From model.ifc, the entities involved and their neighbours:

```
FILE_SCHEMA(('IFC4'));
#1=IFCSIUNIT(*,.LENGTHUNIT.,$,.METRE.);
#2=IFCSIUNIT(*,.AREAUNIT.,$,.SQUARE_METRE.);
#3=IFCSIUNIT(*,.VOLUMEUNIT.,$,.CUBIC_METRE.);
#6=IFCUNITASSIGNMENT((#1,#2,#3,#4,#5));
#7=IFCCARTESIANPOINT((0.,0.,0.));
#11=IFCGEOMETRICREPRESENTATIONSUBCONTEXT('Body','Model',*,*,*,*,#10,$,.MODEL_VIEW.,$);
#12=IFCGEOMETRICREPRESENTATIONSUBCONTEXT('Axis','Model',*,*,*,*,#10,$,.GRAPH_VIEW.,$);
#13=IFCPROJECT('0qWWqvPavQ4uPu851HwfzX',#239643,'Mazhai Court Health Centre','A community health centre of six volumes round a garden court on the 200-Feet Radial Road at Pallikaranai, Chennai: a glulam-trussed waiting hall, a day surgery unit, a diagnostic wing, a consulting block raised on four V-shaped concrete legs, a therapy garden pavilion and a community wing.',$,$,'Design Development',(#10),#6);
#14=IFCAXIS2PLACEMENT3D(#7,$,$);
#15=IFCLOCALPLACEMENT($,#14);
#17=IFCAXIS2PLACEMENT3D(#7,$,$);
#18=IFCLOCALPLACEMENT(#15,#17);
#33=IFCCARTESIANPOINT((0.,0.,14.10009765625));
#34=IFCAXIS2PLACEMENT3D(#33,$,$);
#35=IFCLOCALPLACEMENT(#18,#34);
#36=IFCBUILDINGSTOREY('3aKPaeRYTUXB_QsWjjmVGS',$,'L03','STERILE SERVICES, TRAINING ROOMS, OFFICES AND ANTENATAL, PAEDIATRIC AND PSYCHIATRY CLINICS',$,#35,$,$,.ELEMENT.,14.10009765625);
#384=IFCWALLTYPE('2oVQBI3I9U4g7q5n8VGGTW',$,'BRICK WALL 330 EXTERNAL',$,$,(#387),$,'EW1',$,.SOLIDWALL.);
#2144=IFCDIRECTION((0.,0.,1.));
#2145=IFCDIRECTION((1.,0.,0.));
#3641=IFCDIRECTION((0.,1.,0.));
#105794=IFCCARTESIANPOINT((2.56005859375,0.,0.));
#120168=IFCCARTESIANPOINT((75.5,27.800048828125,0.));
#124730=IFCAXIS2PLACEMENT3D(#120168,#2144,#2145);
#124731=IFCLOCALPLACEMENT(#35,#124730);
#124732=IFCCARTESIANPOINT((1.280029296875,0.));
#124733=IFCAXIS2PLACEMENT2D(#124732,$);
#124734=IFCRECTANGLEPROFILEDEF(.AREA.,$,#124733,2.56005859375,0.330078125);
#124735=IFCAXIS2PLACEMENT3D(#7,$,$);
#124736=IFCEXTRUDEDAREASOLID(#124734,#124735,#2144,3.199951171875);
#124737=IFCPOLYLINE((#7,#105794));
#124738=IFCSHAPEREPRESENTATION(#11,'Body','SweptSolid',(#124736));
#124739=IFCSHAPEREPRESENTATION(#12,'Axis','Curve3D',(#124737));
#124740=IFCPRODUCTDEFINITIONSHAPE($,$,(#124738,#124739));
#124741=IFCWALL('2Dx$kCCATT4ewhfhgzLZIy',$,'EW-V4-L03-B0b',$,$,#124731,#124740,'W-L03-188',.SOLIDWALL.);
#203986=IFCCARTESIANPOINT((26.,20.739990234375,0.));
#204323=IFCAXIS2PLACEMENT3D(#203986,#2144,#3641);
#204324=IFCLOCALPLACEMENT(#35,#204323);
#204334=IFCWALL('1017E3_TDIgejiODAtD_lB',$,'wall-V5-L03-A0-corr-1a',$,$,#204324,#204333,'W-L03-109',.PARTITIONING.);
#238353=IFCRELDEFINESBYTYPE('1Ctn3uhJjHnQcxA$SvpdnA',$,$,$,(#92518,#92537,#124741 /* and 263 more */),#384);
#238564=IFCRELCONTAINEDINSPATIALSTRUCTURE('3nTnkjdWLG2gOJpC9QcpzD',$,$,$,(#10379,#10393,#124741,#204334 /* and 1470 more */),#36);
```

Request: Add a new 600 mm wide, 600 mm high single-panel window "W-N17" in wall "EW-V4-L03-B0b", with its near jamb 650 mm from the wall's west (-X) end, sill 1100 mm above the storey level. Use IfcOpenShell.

```python
import numpy as np
import ifcopenshell
import ifcopenshell.api.feature
import ifcopenshell.api.geometry
import ifcopenshell.api.root
import ifcopenshell.api.spatial
import ifcopenshell.geom
import ifcopenshell.util.element
import ifcopenshell.util.placement
import ifcopenshell.util.representation
import ifcopenshell.util.shape
import ifcopenshell.util.unit

model = ifcopenshell.open("model.ifc")
unit_scale = ifcopenshell.util.unit.calculate_unit_scale(model)
settings = ifcopenshell.geom.settings()


def volume(element):
    """Net volume in cubic metres, openings subtracted."""
    shape = ifcopenshell.geom.create_shape(settings, element)
    return ifcopenshell.util.shape.get_volume(shape.geometry)


wall = model.by_id(124741)
storey = ifcopenshell.util.element.get_container(wall, ifc_class="IfcBuildingStorey")
context = ifcopenshell.util.representation.get_context(model, "Model", "Body", "MODEL_VIEW")
before = volume(wall)

width, height, from_end, sill = 0.6, 0.6, 0.65, 1.1  # metres

# The wall runs along its own X axis, and the end named is its -X end.
wall_shape = ifcopenshell.geom.create_shape(settings, wall)
x, y, z = ifcopenshell.util.shape.get_vertices(wall_shape.geometry).T
start = x.min() + from_end
face, thickness = float(y.min()), float(y.max() - y.min())
wall_matrix = ifcopenshell.util.placement.get_local_placement(wall.ObjectPlacement)
level = ifcopenshell.util.placement.get_local_placement(storey.ObjectPlacement)[2, 3]


def in_wall(x, y):
    """Placement at x, y metres in the wall's axes, at sill height."""
    matrix = wall_matrix.copy()
    matrix[:, 3] = wall_matrix @ np.array([x / unit_scale, y / unit_scale, 0.0, 1.0])
    matrix[2, 3] = level + sill / unit_scale
    return matrix


# Opening: a box that overshoots both wall faces by 50 mm.
opening = ifcopenshell.api.root.create_entity(model, ifc_class="IfcOpeningElement", predefined_type="OPENING")
box = ifcopenshell.api.geometry.add_wall_representation(
    model, context=context, length=width, height=height, thickness=thickness + 0.1
)
ifcopenshell.api.geometry.assign_representation(model, product=opening, representation=box)
ifcopenshell.api.geometry.edit_object_placement(model, product=opening, matrix=in_wall(start, face - 0.05), is_si=False)
ifcopenshell.api.feature.add_feature(model, feature=opening, element=wall)

window = ifcopenshell.api.root.create_entity(model, ifc_class="IfcWindow", name="W-N17", predefined_type="WINDOW")
window.OverallWidth, window.OverallHeight = width / unit_scale, height / unit_scale
window.PartitioningType = "SINGLE_PANEL"
body = ifcopenshell.api.geometry.add_window_representation(
    model,
    context=context,
    overall_width=window.OverallWidth,
    overall_height=window.OverallHeight,
    partition_type="SINGLE_PANEL",
)
ifcopenshell.api.geometry.assign_representation(model, product=window, representation=body)
ifcopenshell.api.spatial.assign_container(model, products=[window], relating_structure=storey)
ifcopenshell.api.feature.add_filling(model, opening=opening, element=window)

# Centre the window in the wall's thickness.
ifcopenshell.api.geometry.edit_object_placement(model, product=window, matrix=in_wall(start, face), is_si=False)
window_shape = ifcopenshell.geom.create_shape(settings, window)
depth = ifcopenshell.util.shape.get_vertices(window_shape.geometry)[:, 1]
offset = face + thickness / 2 - (depth.min() + depth.max()) / 2
ifcopenshell.api.geometry.edit_object_placement(model, product=window, matrix=in_wall(start, offset), is_si=False)

after = volume(wall)

print(f"wall volume {before:.3f} -> {after:.3f} m3")

model.write("model-out.ifc")
```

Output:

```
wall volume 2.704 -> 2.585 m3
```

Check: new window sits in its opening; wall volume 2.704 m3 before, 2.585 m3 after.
